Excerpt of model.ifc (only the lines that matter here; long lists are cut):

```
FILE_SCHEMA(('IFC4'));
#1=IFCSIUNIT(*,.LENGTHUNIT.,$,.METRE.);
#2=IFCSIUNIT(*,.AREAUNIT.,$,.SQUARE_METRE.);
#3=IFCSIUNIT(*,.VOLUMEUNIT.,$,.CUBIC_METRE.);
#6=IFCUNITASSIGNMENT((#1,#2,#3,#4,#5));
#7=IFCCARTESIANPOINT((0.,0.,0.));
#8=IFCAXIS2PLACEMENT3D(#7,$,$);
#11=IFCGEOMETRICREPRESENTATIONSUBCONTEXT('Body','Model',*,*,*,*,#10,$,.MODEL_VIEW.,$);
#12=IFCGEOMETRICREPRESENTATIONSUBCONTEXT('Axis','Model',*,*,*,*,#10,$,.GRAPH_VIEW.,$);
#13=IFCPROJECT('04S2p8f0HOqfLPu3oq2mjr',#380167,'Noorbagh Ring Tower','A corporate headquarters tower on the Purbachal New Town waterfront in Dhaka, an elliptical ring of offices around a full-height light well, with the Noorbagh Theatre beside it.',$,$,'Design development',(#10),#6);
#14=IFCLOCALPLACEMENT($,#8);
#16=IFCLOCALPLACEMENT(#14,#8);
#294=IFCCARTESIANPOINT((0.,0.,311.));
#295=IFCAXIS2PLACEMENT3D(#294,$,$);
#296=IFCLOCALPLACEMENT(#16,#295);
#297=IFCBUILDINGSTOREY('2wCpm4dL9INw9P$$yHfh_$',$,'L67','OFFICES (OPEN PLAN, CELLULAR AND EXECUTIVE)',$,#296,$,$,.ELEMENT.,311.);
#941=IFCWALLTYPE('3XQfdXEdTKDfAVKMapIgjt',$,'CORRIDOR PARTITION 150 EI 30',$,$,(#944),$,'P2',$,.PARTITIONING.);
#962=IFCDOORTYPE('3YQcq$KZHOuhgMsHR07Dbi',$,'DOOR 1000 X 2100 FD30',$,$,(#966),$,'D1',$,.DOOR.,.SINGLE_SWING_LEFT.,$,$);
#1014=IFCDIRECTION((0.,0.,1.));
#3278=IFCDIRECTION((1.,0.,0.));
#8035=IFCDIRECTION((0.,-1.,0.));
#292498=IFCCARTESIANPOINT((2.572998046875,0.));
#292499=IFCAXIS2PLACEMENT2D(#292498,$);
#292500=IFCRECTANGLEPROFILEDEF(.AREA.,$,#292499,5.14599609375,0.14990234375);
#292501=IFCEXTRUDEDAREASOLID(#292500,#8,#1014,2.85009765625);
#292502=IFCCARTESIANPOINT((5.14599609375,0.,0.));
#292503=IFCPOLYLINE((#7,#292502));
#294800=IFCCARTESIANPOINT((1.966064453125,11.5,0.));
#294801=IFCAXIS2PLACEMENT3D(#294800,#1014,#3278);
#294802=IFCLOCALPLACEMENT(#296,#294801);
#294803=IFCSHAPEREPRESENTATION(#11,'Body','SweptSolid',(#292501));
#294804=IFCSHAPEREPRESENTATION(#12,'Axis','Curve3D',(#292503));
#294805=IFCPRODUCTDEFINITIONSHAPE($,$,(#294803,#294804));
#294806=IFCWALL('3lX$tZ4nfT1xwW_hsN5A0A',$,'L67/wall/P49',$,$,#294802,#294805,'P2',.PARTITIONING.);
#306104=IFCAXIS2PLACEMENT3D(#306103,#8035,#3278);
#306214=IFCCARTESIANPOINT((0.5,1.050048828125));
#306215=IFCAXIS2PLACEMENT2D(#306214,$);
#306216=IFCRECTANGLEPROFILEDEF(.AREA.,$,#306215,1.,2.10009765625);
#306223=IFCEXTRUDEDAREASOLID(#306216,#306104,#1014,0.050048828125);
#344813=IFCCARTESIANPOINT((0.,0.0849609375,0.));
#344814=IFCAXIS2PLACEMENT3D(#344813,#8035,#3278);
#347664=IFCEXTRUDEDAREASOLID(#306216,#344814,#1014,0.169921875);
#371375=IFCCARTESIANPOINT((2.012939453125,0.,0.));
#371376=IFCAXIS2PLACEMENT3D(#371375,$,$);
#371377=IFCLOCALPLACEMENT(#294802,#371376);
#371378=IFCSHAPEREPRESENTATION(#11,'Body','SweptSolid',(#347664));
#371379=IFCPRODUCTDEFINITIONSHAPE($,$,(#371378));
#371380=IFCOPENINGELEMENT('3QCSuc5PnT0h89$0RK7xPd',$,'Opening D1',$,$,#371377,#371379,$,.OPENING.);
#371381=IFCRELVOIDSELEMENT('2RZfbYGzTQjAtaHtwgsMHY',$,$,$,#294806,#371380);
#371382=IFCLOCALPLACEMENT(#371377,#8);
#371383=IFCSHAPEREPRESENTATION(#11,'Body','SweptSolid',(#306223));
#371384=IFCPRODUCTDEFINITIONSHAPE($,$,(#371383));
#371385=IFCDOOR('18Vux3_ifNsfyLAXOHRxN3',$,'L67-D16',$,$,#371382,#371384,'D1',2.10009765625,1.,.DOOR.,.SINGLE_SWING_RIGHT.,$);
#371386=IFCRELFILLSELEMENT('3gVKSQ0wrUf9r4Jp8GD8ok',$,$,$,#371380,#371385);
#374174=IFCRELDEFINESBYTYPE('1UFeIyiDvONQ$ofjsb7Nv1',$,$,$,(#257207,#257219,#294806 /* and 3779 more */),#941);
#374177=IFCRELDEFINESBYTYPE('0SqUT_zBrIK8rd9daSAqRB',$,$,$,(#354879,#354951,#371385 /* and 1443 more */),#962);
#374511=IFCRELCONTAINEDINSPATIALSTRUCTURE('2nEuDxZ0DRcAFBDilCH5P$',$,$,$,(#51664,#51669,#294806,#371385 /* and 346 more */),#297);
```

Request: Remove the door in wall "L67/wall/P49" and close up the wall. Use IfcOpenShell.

```python
import ifcopenshell
import ifcopenshell.api.feature
import ifcopenshell.api.root
import ifcopenshell.geom
import ifcopenshell.util.shape

model = ifcopenshell.open("model.ifc")
settings = ifcopenshell.geom.settings()


def volume(element):
    """Net volume in cubic metres, openings subtracted."""
    shape = ifcopenshell.geom.create_shape(settings, element)
    return ifcopenshell.util.shape.get_volume(shape.geometry)


door = model.by_guid("18Vux3_ifNsfyLAXOHRxN3")
opening = door.FillsVoids[0].RelatingOpeningElement
wall = opening.VoidsElements[0].RelatingBuildingElement
before = volume(wall)

ifcopenshell.api.root.remove_product(model, product=door)
ifcopenshell.api.feature.remove_feature(model, feature=opening)

after = volume(wall)

print(f"wall volume {before:.3f} -> {after:.3f} m3")

model.write("model_updated.ifc")
```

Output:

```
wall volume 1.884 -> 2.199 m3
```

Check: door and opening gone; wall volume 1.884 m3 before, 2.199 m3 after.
